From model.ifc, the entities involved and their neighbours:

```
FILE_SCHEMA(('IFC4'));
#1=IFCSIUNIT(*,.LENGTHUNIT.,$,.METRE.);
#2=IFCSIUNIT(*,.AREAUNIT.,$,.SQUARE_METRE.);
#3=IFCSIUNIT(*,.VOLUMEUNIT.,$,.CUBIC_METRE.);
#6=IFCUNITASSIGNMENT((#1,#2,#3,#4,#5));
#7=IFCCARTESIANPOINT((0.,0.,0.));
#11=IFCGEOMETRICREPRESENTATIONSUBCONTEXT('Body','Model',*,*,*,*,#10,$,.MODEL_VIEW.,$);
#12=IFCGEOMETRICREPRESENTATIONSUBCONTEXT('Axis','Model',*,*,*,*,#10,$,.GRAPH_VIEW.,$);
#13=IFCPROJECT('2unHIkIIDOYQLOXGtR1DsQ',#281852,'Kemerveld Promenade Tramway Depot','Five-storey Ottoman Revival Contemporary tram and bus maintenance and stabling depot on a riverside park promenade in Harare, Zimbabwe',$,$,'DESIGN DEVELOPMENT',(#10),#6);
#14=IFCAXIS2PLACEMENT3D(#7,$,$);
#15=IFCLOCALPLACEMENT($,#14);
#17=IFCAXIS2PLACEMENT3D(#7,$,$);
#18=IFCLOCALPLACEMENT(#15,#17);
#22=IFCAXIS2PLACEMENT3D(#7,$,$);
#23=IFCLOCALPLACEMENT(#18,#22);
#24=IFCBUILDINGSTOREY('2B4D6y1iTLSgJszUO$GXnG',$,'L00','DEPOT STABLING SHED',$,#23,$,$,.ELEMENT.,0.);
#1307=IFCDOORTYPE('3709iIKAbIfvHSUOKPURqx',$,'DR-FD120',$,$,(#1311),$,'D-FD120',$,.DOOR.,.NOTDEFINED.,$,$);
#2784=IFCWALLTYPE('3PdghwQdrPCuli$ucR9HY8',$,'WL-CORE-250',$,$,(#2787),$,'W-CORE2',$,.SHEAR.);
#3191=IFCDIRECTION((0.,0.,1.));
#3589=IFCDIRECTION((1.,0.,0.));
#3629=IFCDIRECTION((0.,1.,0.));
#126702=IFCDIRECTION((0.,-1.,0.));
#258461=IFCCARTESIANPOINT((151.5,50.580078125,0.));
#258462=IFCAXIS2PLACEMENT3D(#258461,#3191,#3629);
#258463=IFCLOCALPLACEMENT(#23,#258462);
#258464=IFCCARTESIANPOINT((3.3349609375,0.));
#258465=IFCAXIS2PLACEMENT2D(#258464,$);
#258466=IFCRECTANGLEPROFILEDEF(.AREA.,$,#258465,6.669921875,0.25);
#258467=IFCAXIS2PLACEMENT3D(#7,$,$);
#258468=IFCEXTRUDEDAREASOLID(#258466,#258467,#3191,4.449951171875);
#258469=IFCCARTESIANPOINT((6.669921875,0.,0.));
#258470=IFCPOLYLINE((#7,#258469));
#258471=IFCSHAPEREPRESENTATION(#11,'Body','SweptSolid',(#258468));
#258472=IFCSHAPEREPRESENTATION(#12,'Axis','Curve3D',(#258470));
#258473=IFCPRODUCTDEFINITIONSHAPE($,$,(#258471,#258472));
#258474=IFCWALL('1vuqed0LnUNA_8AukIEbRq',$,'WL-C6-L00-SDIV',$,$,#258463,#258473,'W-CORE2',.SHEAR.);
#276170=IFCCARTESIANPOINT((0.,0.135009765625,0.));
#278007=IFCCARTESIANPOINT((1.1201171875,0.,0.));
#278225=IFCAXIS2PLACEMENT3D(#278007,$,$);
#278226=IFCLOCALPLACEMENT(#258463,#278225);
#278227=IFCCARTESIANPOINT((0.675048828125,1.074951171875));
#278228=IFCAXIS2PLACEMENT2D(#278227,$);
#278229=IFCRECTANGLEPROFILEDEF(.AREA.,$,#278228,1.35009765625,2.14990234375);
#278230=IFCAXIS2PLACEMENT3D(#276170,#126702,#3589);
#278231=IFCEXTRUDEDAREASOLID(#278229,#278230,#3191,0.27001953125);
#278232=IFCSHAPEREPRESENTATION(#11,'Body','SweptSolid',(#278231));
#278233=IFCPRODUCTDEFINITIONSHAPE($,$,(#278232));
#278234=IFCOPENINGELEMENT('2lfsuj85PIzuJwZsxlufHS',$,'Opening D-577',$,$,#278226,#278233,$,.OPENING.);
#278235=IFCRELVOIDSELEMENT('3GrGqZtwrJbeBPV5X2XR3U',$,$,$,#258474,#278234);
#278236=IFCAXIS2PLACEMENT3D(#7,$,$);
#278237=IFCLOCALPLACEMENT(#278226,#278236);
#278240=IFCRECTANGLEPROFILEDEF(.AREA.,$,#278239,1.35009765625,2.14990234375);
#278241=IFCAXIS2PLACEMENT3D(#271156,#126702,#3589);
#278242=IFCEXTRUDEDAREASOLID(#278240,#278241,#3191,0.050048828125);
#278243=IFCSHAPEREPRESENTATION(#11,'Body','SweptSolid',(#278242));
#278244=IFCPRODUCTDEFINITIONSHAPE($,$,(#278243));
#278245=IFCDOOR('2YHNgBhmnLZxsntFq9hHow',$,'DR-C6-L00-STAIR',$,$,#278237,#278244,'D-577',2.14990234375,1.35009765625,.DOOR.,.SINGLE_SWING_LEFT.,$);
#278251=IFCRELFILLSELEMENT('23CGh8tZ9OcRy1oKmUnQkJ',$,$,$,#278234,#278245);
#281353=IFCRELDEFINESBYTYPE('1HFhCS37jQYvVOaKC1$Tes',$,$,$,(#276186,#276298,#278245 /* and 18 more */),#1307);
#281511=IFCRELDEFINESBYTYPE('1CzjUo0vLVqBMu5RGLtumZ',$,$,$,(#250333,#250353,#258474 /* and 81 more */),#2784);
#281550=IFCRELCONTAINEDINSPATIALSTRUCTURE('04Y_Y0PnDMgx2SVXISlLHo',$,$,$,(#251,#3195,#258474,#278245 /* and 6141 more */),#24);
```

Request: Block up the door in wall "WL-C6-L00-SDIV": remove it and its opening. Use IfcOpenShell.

```python
import ifcopenshell
import ifcopenshell.api.feature
import ifcopenshell.api.root
import ifcopenshell.geom
import ifcopenshell.util.shape

model = ifcopenshell.open("model.ifc")
settings = ifcopenshell.geom.settings()


def volume(element):
    """Net volume in cubic metres, openings subtracted."""
    shape = ifcopenshell.geom.create_shape(settings, element)
    return ifcopenshell.util.shape.get_volume(shape.geometry)


door = model.by_guid("2YHNgBhmnLZxsntFq9hHow")
opening = door.FillsVoids[0].RelatingOpeningElement
wall = opening.VoidsElements[0].RelatingBuildingElement
before = volume(wall)

ifcopenshell.api.root.remove_product(model, product=door)
ifcopenshell.api.feature.remove_feature(model, feature=opening)

after = volume(wall)

print(f"wall volume {before:.3f} -> {after:.3f} m3")

model.write("model-out.ifc")
```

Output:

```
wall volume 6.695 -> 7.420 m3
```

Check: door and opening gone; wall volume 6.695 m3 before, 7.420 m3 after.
